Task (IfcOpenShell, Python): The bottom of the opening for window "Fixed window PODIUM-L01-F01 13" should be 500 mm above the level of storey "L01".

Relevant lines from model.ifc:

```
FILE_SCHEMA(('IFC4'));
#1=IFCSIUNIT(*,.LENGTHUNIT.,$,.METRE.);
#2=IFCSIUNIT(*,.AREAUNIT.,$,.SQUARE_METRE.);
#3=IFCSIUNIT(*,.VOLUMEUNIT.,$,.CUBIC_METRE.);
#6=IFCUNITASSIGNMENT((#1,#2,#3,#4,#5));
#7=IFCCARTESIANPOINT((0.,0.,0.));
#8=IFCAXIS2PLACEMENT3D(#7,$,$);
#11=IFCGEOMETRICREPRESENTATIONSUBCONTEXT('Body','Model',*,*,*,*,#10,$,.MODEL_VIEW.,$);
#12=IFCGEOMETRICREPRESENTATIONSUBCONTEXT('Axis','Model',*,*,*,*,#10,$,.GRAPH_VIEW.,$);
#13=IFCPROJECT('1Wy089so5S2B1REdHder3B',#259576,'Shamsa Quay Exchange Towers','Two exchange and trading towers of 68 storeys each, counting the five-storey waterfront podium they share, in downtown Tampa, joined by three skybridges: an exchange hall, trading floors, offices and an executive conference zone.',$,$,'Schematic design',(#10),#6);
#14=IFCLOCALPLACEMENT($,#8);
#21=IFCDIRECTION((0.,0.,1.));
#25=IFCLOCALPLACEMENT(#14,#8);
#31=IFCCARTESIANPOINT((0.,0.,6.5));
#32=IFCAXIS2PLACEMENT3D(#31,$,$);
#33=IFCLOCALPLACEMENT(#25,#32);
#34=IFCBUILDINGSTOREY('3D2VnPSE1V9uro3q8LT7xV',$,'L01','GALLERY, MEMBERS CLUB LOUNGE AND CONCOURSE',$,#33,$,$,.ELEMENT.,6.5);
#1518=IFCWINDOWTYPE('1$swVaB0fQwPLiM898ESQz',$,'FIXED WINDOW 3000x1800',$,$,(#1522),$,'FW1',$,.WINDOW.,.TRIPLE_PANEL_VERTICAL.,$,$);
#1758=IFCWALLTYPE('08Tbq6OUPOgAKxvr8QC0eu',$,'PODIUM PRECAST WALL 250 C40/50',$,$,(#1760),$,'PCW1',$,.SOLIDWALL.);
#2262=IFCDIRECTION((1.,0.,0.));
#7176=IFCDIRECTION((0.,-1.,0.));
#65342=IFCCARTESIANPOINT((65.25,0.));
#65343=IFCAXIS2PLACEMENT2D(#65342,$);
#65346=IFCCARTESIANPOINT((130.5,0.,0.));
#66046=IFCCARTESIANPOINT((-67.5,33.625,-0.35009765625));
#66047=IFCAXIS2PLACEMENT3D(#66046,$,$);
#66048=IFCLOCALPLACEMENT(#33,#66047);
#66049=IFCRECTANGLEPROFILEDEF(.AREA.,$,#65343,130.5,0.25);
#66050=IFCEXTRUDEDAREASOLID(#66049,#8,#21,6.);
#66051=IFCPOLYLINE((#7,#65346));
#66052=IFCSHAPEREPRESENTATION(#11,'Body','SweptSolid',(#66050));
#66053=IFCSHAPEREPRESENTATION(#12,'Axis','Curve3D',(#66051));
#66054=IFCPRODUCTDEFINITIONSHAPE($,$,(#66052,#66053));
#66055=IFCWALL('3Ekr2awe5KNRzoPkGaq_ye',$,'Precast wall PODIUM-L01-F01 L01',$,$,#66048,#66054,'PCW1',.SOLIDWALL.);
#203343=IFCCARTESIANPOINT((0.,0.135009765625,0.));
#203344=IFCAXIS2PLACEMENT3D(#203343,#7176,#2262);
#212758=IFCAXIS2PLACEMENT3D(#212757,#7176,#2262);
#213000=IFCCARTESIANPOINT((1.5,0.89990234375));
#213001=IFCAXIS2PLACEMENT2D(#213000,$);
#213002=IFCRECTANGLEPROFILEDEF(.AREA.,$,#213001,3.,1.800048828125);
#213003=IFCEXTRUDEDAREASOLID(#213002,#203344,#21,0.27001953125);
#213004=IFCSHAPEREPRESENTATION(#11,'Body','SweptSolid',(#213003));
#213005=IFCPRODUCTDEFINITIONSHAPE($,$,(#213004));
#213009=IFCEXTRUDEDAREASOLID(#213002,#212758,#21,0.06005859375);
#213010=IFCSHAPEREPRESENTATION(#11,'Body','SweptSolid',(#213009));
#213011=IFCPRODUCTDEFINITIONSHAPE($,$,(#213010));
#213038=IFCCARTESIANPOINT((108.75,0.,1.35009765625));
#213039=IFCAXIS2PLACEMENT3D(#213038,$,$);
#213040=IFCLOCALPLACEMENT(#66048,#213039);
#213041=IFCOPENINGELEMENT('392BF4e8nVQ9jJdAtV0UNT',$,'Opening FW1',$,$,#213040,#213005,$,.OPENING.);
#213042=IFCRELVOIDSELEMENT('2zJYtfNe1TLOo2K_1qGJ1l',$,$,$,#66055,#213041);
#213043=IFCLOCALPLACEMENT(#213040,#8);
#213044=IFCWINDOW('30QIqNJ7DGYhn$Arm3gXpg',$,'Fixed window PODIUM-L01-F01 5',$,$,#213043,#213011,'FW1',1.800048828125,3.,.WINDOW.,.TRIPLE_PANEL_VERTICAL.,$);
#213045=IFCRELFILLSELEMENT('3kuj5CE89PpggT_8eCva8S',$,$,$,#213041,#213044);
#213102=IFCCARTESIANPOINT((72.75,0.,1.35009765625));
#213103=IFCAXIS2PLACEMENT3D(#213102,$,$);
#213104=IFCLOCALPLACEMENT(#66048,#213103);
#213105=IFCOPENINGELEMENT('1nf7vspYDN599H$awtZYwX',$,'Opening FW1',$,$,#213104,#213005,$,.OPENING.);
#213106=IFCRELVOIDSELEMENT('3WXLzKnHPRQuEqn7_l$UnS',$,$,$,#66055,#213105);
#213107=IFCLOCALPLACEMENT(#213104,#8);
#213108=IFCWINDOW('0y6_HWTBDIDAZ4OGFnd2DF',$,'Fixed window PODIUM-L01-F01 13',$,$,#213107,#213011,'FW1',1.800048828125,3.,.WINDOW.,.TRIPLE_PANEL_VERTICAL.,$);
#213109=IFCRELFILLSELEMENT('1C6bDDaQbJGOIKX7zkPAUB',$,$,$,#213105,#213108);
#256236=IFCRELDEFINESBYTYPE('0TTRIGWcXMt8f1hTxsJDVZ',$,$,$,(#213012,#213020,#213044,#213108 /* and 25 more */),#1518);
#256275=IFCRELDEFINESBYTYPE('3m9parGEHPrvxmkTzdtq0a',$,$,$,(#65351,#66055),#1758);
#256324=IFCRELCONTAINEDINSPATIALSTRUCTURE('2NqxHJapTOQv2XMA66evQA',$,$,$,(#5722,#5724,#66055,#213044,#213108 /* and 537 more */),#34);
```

```python
import numpy as np
import ifcopenshell
import ifcopenshell.api.geometry
import ifcopenshell.geom
import ifcopenshell.util.element
import ifcopenshell.util.placement
import ifcopenshell.util.shape
import ifcopenshell.util.unit

model = ifcopenshell.open("model.ifc")
unit_scale = ifcopenshell.util.unit.calculate_unit_scale(model)

window = model.by_guid("0y6_HWTBDIDAZ4OGFnd2DF")
opening = window.FillsVoids[0].RelatingOpeningElement
storey = ifcopenshell.util.element.get_container(window, ifc_class="IfcBuildingStorey")
level = ifcopenshell.util.placement.get_local_placement(storey.ObjectPlacement)[2, 3]

# The opening's origin need not be at the sill, so measure its lowest point.
shape = ifcopenshell.geom.create_shape(ifcopenshell.geom.settings(), opening)
bottom = ifcopenshell.util.shape.get_shape_bottom_elevation(shape, shape.geometry) / unit_scale
dz = level + 0.5 / unit_scale - bottom

shift = np.array([0.0, 0.0, dz])
# The window is placed relative to its opening, so it follows when the opening moves.
matrix = ifcopenshell.util.placement.get_local_placement(opening.ObjectPlacement)
matrix[:3, 3] += shift
ifcopenshell.api.geometry.edit_object_placement(
    model, product=opening, matrix=matrix, is_si=False, should_transform_children=True
)

print(f"moved by {dz * unit_scale:+.3f} m")

model.write("model-out.ifc")
```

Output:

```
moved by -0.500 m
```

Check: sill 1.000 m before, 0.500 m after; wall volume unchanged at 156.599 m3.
